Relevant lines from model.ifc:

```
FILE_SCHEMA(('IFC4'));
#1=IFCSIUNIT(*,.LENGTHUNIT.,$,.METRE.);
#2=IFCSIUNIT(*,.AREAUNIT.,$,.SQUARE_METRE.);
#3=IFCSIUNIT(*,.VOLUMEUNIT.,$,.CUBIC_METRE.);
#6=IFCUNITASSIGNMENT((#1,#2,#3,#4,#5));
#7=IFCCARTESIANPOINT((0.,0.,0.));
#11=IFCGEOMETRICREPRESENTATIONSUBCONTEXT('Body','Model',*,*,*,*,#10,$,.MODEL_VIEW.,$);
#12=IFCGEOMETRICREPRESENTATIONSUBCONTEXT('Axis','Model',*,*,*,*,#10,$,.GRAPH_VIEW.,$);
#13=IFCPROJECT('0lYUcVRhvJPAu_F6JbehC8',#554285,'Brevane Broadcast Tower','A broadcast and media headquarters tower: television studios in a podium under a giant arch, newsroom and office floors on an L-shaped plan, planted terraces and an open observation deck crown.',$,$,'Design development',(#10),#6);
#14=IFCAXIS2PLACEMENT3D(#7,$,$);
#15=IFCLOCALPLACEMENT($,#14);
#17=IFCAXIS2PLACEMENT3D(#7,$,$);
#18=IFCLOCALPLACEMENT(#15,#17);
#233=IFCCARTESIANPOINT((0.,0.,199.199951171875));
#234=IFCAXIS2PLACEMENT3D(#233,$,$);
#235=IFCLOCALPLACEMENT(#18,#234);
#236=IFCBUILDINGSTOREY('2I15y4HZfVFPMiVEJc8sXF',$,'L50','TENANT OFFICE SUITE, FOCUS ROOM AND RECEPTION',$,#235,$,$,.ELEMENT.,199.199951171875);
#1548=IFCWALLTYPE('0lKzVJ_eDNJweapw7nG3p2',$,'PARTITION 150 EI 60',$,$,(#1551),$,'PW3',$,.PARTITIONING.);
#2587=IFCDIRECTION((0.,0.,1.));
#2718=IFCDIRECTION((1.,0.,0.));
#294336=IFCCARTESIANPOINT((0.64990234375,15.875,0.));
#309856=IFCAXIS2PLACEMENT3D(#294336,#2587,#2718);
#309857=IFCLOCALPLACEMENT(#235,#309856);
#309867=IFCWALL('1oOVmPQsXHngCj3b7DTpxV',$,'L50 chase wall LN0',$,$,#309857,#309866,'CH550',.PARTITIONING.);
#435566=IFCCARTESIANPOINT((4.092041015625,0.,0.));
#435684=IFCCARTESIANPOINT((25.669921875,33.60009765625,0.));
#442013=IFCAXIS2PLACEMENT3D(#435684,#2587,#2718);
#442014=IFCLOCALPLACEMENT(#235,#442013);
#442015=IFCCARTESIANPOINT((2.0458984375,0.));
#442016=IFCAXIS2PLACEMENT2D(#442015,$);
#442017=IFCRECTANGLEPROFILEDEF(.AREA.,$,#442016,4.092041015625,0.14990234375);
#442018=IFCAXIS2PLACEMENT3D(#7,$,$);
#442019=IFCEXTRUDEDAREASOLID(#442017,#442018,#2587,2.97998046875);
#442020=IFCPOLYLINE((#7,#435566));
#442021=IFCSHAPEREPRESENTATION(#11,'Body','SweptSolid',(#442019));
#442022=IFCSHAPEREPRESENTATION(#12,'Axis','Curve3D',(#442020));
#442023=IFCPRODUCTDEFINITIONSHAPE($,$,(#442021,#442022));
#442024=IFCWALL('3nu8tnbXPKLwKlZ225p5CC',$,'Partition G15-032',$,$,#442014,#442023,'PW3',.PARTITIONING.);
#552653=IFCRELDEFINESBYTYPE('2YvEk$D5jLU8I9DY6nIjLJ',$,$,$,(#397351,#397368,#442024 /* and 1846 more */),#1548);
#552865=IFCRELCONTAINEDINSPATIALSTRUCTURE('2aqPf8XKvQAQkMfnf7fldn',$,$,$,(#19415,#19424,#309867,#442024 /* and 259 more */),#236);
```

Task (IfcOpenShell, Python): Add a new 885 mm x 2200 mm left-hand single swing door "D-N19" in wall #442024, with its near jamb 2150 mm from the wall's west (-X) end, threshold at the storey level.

```python
import numpy as np
import ifcopenshell
import ifcopenshell.api.feature
import ifcopenshell.api.geometry
import ifcopenshell.api.root
import ifcopenshell.api.spatial
import ifcopenshell.geom
import ifcopenshell.util.element
import ifcopenshell.util.placement
import ifcopenshell.util.representation
import ifcopenshell.util.shape
import ifcopenshell.util.unit

model = ifcopenshell.open("model.ifc")
unit_scale = ifcopenshell.util.unit.calculate_unit_scale(model)
settings = ifcopenshell.geom.settings()


def volume(element):
    """Net volume in cubic metres, openings subtracted."""
    shape = ifcopenshell.geom.create_shape(settings, element)
    return ifcopenshell.util.shape.get_volume(shape.geometry)


wall = model.by_guid("3nu8tnbXPKLwKlZ225p5CC")
storey = ifcopenshell.util.element.get_container(wall, ifc_class="IfcBuildingStorey")
context = ifcopenshell.util.representation.get_context(model, "Model", "Body", "MODEL_VIEW")
before = volume(wall)

width, height, from_end, sill = 0.885, 2.2, 2.15, 0.0  # metres

# The wall runs along its own X axis, and the end named is its -X end.
wall_shape = ifcopenshell.geom.create_shape(settings, wall)
x, y, z = ifcopenshell.util.shape.get_vertices(wall_shape.geometry).T
start = x.min() + from_end
face, thickness = float(y.min()), float(y.max() - y.min())
wall_matrix = ifcopenshell.util.placement.get_local_placement(wall.ObjectPlacement)
level = ifcopenshell.util.placement.get_local_placement(storey.ObjectPlacement)[2, 3]


def in_wall(x, y):
    """Placement at x, y metres in the wall's axes, at sill height."""
    matrix = wall_matrix.copy()
    matrix[:, 3] = wall_matrix @ np.array([x / unit_scale, y / unit_scale, 0.0, 1.0])
    matrix[2, 3] = level + sill / unit_scale
    return matrix


# Opening: a box that overshoots both wall faces by 50 mm.
opening = ifcopenshell.api.root.create_entity(model, ifc_class="IfcOpeningElement", predefined_type="OPENING")
box = ifcopenshell.api.geometry.add_wall_representation(
    model, context=context, length=width, height=height, thickness=thickness + 0.1
)
ifcopenshell.api.geometry.assign_representation(model, product=opening, representation=box)
ifcopenshell.api.geometry.edit_object_placement(model, product=opening, matrix=in_wall(start, face - 0.05), is_si=False)
ifcopenshell.api.feature.add_feature(model, feature=opening, element=wall)

door = ifcopenshell.api.root.create_entity(model, ifc_class="IfcDoor", name="D-N19", predefined_type="DOOR")
door.OverallWidth, door.OverallHeight = width / unit_scale, height / unit_scale
door.OperationType = "SINGLE_SWING_LEFT"
body = ifcopenshell.api.geometry.add_door_representation(
    model,
    context=context,
    overall_width=door.OverallWidth,
    overall_height=door.OverallHeight,
    operation_type="SINGLE_SWING_LEFT",
    lining_properties={"LiningDepth": thickness / unit_scale, "ThresholdDepth": thickness / unit_scale},
)
ifcopenshell.api.geometry.assign_representation(model, product=door, representation=body)
ifcopenshell.api.spatial.assign_container(model, products=[door], relating_structure=storey)
ifcopenshell.api.feature.add_filling(model, opening=opening, element=door)

# The lining spans the wall, so the door starts at the wall face.
ifcopenshell.api.geometry.edit_object_placement(model, product=door, matrix=in_wall(start, face), is_si=False)

after = volume(wall)

print(f"wall volume {before:.3f} -> {after:.3f} m3")

model.write("model-out.ifc")
```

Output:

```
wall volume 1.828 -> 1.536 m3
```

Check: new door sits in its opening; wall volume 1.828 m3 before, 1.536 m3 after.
